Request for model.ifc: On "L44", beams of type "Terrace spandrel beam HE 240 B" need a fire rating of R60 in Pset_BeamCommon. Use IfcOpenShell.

First a look at what the model holds.

```python
import ifcopenshell
import ifcopenshell.util.element

model = ifcopenshell.open("model.ifc")
print(model.schema)
storey = next(s for s in model.by_type("IfcBuildingStorey") if s.Name == "L44")
beams = [e for e in ifcopenshell.util.element.get_decomposition(storey) if e.is_a("IfcBeam")]
seen = {}
for e in beams:
    element_type = ifcopenshell.util.element.get_type(e)
    key = (element_type.Name if element_type != e and element_type else None, ifcopenshell.util.element.get_pset(e, "Pset_BeamCommon", "FireRating"))
    seen[key] = seen.get(key, 0) + 1
for (name, value), count in sorted(seen.items(), key=str):
    print(count, "x", name, "|", value)
```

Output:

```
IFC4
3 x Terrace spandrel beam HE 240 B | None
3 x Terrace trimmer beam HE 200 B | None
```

```python
import ifcopenshell
import ifcopenshell.api.pset
import ifcopenshell.util.element

model = ifcopenshell.open("model.ifc")

storey = next(s for s in model.by_type("IfcBuildingStorey") if s.Name == "L44")
beams = [e for e in ifcopenshell.util.element.get_decomposition(storey) if e.is_a("IfcBeam")]

count = 0
for e in beams:
    element_type = ifcopenshell.util.element.get_type(e)
    if element_type in (None, e) or element_type.Name != "Terrace spandrel beam HE 240 B":
        continue
    found = ifcopenshell.util.element.get_pset(e, "Pset_BeamCommon", should_inherit=False)
    if found:
        pset = model.by_id(found["id"])
        if len(ifcopenshell.util.element.get_elements_by_pset(pset)) > 1:
            pset = ifcopenshell.api.pset.unshare_pset(model, products=[e], pset=pset)[0]
    else:
        pset = ifcopenshell.api.pset.add_pset(model, product=e, name="Pset_BeamCommon")
    ifcopenshell.api.pset.edit_pset(model, pset=pset, properties={"FireRating": "R60"})
    count += 1

print(count, "beams updated")

model.write("model_v2.ifc")
```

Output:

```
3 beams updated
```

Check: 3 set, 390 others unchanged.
